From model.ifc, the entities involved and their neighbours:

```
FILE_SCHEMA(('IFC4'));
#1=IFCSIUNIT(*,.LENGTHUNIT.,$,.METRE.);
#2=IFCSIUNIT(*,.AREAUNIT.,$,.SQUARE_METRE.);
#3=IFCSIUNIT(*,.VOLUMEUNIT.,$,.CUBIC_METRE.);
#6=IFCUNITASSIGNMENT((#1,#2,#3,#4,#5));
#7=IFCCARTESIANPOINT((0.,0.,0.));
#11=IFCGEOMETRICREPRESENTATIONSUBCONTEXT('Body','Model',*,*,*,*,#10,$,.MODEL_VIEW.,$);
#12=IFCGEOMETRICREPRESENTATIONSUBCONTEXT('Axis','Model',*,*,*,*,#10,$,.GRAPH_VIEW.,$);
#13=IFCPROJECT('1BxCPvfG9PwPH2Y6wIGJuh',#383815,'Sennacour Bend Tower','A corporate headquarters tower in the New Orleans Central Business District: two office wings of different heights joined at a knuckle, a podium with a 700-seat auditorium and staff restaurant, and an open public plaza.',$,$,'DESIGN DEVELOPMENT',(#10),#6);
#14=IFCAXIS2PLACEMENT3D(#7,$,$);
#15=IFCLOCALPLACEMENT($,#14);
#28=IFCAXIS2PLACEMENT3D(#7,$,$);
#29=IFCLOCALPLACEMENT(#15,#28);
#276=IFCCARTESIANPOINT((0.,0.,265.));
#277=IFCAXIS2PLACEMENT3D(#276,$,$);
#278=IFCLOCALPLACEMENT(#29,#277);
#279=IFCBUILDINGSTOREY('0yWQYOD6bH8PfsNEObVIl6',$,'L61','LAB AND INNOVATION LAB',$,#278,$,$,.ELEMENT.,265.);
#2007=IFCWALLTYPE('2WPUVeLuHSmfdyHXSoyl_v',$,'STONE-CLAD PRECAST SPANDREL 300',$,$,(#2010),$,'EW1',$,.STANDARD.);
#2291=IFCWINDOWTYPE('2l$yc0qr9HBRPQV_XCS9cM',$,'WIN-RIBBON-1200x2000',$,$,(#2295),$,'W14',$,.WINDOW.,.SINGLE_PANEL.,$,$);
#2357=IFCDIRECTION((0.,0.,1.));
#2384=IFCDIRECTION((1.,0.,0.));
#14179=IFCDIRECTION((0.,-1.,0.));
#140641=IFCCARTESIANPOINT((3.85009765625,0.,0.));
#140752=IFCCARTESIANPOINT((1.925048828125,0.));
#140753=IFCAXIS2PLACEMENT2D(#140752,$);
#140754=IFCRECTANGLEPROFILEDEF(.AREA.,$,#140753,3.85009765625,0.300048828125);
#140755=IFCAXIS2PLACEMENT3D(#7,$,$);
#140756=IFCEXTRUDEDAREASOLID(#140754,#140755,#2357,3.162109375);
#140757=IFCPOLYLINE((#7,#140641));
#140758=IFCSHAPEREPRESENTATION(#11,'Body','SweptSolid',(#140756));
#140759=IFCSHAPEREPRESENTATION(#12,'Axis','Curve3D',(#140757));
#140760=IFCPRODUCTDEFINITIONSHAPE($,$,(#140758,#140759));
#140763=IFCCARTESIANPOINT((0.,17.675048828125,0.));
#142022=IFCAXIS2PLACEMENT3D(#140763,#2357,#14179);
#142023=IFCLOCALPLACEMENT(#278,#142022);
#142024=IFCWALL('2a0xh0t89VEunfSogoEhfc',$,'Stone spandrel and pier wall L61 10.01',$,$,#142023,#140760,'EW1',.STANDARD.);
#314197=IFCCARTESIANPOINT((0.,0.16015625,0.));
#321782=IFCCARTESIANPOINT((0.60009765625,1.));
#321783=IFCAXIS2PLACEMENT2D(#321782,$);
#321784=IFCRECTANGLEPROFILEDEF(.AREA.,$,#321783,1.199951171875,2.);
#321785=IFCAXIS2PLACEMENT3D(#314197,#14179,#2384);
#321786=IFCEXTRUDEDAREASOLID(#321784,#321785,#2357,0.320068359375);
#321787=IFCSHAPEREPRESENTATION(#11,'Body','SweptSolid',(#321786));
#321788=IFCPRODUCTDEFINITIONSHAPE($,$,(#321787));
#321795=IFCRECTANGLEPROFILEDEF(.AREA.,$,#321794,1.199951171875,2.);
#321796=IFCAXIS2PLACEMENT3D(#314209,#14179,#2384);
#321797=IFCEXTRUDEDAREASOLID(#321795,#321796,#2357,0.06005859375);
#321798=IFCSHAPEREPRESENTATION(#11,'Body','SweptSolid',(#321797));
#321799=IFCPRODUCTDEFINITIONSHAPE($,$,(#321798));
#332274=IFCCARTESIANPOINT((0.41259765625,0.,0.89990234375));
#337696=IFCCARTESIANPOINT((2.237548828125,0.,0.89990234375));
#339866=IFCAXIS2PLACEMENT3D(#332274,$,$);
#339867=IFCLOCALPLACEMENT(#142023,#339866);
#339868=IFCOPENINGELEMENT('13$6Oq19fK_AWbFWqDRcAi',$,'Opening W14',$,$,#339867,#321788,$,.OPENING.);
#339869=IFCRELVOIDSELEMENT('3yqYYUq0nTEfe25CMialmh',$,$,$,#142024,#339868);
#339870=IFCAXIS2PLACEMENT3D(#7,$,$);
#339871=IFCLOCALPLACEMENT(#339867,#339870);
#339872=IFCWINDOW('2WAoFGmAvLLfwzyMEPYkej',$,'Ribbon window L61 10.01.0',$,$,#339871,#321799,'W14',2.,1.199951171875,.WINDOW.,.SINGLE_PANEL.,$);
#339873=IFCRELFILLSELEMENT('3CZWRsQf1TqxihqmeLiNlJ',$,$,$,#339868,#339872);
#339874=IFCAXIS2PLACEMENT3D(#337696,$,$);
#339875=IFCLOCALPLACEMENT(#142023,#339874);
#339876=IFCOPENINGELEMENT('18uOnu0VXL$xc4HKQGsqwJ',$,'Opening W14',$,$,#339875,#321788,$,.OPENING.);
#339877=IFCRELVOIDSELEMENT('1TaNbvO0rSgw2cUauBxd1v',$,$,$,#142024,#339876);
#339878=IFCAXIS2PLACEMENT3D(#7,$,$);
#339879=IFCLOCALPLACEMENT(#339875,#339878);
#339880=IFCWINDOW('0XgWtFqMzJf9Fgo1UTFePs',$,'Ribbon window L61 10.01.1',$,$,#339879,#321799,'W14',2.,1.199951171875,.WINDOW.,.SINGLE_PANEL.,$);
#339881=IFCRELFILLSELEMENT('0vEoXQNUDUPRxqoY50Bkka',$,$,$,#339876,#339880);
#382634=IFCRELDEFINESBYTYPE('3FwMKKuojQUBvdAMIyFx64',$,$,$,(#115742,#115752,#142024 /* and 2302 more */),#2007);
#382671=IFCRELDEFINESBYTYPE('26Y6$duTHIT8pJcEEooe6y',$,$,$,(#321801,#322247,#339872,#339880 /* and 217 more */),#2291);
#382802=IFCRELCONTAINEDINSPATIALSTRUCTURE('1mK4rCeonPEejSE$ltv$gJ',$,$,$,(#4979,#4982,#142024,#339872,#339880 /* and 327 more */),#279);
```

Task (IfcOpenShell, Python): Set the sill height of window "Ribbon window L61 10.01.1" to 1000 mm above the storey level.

```python
import numpy as np
import ifcopenshell
import ifcopenshell.api.geometry
import ifcopenshell.geom
import ifcopenshell.util.element
import ifcopenshell.util.placement
import ifcopenshell.util.shape
import ifcopenshell.util.unit

model = ifcopenshell.open("model.ifc")
unit_scale = ifcopenshell.util.unit.calculate_unit_scale(model)

window = model.by_guid("0XgWtFqMzJf9Fgo1UTFePs")
opening = window.FillsVoids[0].RelatingOpeningElement
storey = ifcopenshell.util.element.get_container(window, ifc_class="IfcBuildingStorey")
level = ifcopenshell.util.placement.get_local_placement(storey.ObjectPlacement)[2, 3]

# The opening's origin need not be at the sill, so measure its lowest point.
shape = ifcopenshell.geom.create_shape(ifcopenshell.geom.settings(), opening)
bottom = ifcopenshell.util.shape.get_shape_bottom_elevation(shape, shape.geometry) / unit_scale
dz = level + 1 / unit_scale - bottom

shift = np.array([0.0, 0.0, dz])
# The window is placed relative to its opening, so it follows when the opening moves.
matrix = ifcopenshell.util.placement.get_local_placement(opening.ObjectPlacement)
matrix[:3, 3] += shift
ifcopenshell.api.geometry.edit_object_placement(
    model, product=opening, matrix=matrix, is_si=False, should_transform_children=True
)

print(f"moved by {dz * unit_scale:+.3f} m")

model.write("model_edited.ifc")
```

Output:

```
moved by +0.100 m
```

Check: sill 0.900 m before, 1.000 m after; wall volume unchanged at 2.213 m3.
